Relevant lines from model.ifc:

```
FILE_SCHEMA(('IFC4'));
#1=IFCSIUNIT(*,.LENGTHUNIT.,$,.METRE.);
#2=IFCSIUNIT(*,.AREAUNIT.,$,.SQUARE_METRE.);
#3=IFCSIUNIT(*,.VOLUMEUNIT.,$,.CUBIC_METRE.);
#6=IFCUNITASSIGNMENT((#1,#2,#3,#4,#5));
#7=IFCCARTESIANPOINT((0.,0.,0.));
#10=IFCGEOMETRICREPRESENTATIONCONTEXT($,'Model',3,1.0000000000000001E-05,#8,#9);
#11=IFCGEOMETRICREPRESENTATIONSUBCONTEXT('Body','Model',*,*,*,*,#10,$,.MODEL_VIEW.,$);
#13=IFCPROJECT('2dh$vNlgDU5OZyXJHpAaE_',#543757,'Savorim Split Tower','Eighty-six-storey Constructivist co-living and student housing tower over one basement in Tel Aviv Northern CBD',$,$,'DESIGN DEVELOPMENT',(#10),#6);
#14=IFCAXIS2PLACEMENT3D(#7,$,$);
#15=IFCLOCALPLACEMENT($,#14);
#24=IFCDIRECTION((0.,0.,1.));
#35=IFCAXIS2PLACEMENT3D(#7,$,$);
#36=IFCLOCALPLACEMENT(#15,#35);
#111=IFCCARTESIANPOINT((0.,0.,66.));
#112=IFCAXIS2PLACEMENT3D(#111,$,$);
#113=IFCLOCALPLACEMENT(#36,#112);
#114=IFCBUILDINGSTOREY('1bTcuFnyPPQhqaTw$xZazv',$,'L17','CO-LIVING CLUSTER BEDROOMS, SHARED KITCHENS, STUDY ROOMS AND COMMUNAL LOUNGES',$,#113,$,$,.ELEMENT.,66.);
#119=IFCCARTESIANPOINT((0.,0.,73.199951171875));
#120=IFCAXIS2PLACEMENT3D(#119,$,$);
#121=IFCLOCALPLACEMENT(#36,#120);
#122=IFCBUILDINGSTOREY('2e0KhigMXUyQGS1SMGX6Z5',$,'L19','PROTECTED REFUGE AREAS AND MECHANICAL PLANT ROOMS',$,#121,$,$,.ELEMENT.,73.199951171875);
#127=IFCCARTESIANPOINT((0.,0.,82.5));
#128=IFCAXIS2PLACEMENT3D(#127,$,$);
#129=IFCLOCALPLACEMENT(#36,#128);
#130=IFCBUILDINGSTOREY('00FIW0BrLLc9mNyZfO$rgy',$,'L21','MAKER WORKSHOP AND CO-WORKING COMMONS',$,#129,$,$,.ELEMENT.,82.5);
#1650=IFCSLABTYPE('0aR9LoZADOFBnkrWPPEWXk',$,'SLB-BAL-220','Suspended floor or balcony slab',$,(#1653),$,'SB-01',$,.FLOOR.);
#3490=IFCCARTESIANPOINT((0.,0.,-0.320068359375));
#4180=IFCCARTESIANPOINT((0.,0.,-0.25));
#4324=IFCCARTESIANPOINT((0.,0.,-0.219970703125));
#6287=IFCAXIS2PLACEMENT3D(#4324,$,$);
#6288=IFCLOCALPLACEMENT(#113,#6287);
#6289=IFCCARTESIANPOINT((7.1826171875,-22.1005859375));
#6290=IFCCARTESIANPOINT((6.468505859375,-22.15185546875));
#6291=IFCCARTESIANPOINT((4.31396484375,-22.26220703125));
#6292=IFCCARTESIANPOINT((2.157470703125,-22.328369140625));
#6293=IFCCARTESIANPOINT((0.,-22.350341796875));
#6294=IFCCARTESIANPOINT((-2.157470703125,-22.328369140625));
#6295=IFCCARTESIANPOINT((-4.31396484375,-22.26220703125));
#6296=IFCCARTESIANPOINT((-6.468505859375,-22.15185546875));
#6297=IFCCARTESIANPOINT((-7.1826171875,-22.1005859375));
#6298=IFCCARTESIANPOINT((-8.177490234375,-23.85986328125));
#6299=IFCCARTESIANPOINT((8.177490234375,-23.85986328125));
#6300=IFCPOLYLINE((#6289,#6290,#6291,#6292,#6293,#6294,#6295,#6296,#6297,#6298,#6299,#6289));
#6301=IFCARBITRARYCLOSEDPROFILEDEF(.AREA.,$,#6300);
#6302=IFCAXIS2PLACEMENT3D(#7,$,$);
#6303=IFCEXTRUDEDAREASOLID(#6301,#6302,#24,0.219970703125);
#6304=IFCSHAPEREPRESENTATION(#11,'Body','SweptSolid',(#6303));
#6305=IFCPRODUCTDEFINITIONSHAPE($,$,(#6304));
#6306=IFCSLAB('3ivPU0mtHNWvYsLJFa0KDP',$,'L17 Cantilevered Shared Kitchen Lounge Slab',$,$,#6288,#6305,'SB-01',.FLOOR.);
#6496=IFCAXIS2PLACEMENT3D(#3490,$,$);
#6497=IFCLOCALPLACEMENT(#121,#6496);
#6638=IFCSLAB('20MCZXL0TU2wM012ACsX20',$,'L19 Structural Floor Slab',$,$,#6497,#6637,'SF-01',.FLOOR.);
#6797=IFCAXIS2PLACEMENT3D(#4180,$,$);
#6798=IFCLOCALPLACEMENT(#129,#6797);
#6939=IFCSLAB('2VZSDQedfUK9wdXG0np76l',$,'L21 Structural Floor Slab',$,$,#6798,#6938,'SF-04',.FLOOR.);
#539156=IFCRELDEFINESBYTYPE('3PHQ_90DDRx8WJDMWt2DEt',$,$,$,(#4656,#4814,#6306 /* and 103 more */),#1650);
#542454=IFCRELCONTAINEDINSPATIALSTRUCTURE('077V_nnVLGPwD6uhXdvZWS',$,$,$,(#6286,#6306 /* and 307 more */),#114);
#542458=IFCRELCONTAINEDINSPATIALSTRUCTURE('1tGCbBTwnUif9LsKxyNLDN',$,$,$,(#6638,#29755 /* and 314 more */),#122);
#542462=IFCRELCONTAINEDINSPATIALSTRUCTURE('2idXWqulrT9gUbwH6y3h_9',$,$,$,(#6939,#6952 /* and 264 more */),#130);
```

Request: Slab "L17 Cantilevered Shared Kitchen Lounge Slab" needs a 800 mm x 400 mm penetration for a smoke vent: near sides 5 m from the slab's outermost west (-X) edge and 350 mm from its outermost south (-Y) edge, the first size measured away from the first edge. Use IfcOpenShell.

```python
import numpy as np
import ifcopenshell
import ifcopenshell.api.feature
import ifcopenshell.api.geometry
import ifcopenshell.api.root
import ifcopenshell.geom
import ifcopenshell.util.placement
import ifcopenshell.util.representation
import ifcopenshell.util.shape
import ifcopenshell.util.unit

model = ifcopenshell.open("model.ifc")
unit_scale = ifcopenshell.util.unit.calculate_unit_scale(model)
settings = ifcopenshell.geom.settings()


def volume(element):
    """Net volume in cubic metres, openings subtracted."""
    shape = ifcopenshell.geom.create_shape(settings, element)
    return ifcopenshell.util.shape.get_volume(shape.geometry)


slab = model.by_guid("3ivPU0mtHNWvYsLJFa0KDP")
before = volume(slab)

# Extent in the slab's own axes, in metres. The edges named are its -X and -Y sides.
slab_shape = ifcopenshell.geom.create_shape(settings, slab)
vertices = ifcopenshell.util.shape.get_vertices(slab_shape.geometry)
x_min, y_min, bottom = vertices.min(axis=0)
top = vertices[:, 2].max()

opening = ifcopenshell.api.root.create_entity(model, ifc_class="IfcOpeningElement", name="Smoke vent opening", predefined_type="OPENING")
context = ifcopenshell.util.representation.get_context(model, "Model", "Body", "MODEL_VIEW")
width, depth = 0.8, 0.4
outline = [(0.0, 0.0), (width, 0.0), (width, depth), (0.0, depth), (0.0, 0.0)]
# Overshoot both faces by 50 mm so the cut is clean.
shape = ifcopenshell.api.geometry.add_slab_representation(
    model, context=context, depth=top - bottom + 0.1, polyline=outline
)
ifcopenshell.api.geometry.assign_representation(model, product=opening, representation=shape)

matrix = ifcopenshell.util.placement.get_local_placement(slab.ObjectPlacement)
matrix[:, 3] = matrix @ np.append(np.array([x_min + 5, y_min + 0.35, bottom - 0.05]) / unit_scale, 1.0)
ifcopenshell.api.geometry.edit_object_placement(model, product=opening, matrix=matrix, is_si=False)
ifcopenshell.api.feature.add_feature(model, feature=opening, element=slab)

after = volume(slab)

print(f"slab volume {before:.3f} -> {after:.3f} m3")

model.write("model_v2.ifc")
```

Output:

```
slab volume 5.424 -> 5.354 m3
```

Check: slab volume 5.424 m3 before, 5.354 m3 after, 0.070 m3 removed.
